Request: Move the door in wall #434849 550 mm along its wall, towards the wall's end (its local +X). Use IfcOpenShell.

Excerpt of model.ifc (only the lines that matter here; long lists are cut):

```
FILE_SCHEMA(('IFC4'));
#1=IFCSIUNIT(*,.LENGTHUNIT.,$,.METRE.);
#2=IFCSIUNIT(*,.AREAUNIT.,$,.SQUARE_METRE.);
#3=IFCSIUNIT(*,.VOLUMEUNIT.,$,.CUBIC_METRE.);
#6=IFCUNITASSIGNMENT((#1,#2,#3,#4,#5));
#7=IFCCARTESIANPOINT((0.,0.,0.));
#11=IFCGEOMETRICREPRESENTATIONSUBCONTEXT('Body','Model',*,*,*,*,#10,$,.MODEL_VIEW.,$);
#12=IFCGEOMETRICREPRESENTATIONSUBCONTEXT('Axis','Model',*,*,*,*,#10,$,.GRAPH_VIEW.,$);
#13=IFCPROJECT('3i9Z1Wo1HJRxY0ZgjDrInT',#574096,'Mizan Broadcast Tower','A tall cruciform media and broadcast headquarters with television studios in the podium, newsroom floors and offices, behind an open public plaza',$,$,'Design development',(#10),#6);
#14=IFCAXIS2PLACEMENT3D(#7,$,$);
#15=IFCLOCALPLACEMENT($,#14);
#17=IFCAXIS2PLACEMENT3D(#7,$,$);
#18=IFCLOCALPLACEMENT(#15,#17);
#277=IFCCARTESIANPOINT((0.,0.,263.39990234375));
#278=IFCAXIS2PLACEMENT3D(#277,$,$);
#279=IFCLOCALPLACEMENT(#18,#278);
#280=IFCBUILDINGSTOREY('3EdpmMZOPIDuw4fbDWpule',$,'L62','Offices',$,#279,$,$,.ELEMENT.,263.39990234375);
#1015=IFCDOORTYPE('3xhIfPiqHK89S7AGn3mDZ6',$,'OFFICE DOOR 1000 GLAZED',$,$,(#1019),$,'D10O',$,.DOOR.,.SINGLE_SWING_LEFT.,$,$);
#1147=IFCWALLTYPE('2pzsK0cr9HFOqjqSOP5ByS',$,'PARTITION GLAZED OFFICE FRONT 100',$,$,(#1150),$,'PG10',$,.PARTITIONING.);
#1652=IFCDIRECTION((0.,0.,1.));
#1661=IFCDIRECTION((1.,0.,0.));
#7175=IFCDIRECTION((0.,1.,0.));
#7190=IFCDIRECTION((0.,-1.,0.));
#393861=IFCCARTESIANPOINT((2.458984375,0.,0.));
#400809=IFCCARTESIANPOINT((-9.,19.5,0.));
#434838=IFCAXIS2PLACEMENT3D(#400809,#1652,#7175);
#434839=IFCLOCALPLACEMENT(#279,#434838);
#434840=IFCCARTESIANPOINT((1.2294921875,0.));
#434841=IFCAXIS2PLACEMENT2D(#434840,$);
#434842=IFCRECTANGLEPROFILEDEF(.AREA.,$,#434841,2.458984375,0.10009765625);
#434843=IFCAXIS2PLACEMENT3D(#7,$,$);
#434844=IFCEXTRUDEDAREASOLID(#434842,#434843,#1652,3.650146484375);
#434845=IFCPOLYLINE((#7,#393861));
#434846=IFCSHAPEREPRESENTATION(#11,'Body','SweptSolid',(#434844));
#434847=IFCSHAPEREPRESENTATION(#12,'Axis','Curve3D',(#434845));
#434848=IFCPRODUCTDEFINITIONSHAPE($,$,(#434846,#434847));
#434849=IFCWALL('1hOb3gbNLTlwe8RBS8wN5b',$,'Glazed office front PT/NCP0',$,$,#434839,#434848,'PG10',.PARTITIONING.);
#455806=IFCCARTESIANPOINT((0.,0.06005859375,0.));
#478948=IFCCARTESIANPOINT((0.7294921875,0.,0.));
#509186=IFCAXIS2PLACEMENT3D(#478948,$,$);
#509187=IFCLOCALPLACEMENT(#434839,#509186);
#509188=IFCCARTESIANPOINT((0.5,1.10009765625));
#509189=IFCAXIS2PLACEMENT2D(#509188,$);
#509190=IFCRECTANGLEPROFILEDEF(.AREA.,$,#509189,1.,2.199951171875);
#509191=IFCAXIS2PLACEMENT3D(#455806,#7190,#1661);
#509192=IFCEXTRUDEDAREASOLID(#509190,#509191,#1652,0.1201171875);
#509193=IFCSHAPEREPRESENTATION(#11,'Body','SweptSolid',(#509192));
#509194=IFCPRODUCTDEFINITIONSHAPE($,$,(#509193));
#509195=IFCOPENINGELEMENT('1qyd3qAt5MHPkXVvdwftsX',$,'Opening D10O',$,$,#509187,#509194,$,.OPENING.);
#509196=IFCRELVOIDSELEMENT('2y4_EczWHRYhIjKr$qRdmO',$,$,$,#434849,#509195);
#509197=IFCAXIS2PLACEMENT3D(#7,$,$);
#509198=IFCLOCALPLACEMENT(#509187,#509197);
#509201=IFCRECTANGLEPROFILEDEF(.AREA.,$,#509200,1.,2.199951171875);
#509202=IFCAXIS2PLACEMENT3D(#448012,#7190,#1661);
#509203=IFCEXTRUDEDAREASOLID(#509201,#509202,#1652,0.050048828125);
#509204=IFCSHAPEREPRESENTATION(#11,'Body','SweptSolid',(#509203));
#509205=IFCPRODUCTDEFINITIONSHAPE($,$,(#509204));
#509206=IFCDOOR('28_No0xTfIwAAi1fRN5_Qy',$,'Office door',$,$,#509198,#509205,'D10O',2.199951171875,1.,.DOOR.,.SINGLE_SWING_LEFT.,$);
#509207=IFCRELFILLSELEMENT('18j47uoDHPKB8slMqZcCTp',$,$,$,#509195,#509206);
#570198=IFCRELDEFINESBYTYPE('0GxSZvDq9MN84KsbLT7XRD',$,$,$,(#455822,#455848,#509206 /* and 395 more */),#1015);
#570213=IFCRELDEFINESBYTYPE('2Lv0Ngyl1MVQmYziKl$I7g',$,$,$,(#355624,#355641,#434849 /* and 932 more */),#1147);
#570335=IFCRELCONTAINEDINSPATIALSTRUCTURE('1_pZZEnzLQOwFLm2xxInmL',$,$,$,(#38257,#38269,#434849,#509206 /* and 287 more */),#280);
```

```python
import ifcopenshell
import ifcopenshell.api.geometry
import ifcopenshell.util.placement
import ifcopenshell.util.unit

model = ifcopenshell.open("model.ifc")
unit_scale = ifcopenshell.util.unit.calculate_unit_scale(model)

door = model.by_id(509206)
opening = door.FillsVoids[0].RelatingOpeningElement
wall = opening.VoidsElements[0].RelatingBuildingElement

wall_matrix = ifcopenshell.util.placement.get_local_placement(wall.ObjectPlacement)
shift = wall_matrix[:3, 0] * 0.55 / unit_scale
before = ifcopenshell.util.placement.get_local_placement(door.ObjectPlacement)[:3, 3].copy()

# The door is placed relative to its opening, so it follows when the opening moves.
matrix = ifcopenshell.util.placement.get_local_placement(opening.ObjectPlacement)
matrix[:3, 3] += shift
ifcopenshell.api.geometry.edit_object_placement(
    model, product=opening, matrix=matrix, is_si=False, should_transform_children=True
)

after = ifcopenshell.util.placement.get_local_placement(door.ObjectPlacement)[:3, 3]
print("door moved by", (after - before).round(3) + 0.0)

model.write("model_edited.ifc")
```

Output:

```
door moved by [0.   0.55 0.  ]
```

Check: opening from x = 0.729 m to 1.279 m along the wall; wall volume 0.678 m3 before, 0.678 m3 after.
